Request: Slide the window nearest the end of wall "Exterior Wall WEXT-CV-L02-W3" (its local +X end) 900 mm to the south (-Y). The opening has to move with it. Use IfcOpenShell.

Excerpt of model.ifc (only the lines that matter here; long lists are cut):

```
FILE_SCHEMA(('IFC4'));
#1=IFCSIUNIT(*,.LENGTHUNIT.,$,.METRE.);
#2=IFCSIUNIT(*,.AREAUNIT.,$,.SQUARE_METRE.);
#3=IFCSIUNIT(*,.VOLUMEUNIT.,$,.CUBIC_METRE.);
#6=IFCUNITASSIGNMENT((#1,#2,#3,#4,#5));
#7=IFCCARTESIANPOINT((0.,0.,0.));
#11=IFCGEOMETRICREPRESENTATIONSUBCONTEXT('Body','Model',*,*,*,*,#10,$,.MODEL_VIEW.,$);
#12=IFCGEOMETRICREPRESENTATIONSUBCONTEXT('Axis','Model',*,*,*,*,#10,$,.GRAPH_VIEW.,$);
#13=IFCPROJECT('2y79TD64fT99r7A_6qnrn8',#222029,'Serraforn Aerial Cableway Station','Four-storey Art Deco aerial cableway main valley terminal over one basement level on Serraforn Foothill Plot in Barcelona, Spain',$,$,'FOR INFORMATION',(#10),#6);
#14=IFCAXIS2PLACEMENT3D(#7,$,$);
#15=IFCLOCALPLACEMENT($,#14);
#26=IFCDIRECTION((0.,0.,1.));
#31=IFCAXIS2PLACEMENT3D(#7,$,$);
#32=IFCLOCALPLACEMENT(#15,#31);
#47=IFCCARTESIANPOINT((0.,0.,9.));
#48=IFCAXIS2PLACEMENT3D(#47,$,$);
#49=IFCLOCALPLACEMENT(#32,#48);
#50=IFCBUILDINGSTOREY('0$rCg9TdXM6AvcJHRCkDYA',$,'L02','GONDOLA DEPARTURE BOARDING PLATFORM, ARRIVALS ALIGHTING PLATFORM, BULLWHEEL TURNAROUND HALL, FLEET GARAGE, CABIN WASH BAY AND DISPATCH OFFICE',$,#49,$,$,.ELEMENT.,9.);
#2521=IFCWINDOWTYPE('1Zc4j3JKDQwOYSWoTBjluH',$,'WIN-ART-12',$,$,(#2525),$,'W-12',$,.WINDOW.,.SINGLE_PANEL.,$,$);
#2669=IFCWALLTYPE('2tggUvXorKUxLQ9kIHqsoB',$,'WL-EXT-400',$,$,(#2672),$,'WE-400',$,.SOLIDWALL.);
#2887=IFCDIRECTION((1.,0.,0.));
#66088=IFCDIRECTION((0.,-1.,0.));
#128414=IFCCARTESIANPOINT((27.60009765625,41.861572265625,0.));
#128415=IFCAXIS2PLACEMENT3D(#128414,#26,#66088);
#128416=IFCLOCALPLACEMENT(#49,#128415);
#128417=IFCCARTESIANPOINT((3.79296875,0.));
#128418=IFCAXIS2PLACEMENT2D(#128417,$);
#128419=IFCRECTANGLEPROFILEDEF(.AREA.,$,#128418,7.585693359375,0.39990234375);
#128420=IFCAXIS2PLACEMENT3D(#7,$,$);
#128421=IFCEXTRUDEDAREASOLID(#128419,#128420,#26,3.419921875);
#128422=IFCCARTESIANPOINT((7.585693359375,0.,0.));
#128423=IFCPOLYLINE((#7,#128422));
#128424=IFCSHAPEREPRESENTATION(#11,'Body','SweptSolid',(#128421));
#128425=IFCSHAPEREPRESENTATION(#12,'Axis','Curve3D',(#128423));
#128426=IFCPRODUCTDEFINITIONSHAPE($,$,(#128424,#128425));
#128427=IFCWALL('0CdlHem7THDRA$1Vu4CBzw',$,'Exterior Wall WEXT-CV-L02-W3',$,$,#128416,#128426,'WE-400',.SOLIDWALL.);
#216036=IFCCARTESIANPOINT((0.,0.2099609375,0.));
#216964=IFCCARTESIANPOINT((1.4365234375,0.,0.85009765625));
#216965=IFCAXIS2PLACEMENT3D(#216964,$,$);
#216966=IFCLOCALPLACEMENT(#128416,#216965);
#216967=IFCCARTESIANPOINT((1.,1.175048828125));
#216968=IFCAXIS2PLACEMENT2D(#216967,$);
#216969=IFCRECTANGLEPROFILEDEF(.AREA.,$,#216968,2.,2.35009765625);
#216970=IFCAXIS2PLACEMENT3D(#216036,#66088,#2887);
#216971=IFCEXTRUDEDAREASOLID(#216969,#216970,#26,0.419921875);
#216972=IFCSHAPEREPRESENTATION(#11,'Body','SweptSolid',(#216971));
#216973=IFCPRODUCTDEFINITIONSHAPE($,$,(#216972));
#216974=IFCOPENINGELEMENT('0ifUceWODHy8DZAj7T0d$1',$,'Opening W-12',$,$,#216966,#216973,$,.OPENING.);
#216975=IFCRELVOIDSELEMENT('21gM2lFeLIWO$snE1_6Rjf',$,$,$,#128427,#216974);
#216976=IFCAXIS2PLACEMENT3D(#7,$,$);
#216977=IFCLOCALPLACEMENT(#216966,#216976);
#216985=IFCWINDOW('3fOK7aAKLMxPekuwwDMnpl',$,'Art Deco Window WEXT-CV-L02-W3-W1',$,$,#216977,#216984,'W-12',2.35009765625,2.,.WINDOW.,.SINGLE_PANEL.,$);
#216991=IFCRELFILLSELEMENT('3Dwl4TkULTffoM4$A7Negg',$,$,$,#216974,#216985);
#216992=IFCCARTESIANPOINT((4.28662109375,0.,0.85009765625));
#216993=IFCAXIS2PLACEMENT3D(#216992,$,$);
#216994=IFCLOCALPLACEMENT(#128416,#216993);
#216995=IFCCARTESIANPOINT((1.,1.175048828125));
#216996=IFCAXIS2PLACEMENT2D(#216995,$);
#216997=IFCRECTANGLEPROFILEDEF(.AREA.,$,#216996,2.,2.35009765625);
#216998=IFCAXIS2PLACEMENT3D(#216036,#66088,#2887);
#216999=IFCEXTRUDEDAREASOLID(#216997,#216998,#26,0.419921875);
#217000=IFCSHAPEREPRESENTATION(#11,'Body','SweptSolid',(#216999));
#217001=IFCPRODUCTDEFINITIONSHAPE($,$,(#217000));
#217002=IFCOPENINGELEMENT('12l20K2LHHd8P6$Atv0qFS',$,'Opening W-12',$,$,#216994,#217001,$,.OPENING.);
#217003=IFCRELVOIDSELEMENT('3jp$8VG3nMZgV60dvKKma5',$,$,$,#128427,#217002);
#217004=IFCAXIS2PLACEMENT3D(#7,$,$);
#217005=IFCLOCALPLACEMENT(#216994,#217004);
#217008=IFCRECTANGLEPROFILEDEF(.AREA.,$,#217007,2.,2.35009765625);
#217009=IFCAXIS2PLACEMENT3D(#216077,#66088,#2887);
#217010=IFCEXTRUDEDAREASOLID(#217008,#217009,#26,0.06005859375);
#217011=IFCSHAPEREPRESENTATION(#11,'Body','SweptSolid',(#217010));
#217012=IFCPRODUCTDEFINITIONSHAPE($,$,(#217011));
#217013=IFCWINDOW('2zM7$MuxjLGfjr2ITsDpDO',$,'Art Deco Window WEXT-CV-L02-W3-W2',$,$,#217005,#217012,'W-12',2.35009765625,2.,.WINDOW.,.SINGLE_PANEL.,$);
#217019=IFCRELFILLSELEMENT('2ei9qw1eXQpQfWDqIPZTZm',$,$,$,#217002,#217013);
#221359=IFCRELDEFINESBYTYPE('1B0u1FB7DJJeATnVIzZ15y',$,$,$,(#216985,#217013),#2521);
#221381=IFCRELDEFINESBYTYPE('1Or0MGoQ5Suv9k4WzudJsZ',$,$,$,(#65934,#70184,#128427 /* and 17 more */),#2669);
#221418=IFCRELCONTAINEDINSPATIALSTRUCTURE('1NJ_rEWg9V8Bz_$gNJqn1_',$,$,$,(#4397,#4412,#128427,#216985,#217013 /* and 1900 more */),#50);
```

```python
import ifcopenshell
import ifcopenshell.api.geometry
import ifcopenshell.util.placement
import ifcopenshell.util.unit

model = ifcopenshell.open("model.ifc")
unit_scale = ifcopenshell.util.unit.calculate_unit_scale(model)

window = model.by_id(217013)
opening = window.FillsVoids[0].RelatingOpeningElement
wall = opening.VoidsElements[0].RelatingBuildingElement

wall_matrix = ifcopenshell.util.placement.get_local_placement(wall.ObjectPlacement)
shift = wall_matrix[:3, 0] * 0.9 / unit_scale
before = ifcopenshell.util.placement.get_local_placement(window.ObjectPlacement)[:3, 3].copy()

# The window is placed relative to its opening, so it follows when the opening moves.
matrix = ifcopenshell.util.placement.get_local_placement(opening.ObjectPlacement)
matrix[:3, 3] += shift
ifcopenshell.api.geometry.edit_object_placement(
    model, product=opening, matrix=matrix, is_si=False, should_transform_children=True
)

after = ifcopenshell.util.placement.get_local_placement(window.ObjectPlacement)[:3, 3]
print("window moved by", (after - before).round(3) + 0.0)

model.write("model-out.ifc")
```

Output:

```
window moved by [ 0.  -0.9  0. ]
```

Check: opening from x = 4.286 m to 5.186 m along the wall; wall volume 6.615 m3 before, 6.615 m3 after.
